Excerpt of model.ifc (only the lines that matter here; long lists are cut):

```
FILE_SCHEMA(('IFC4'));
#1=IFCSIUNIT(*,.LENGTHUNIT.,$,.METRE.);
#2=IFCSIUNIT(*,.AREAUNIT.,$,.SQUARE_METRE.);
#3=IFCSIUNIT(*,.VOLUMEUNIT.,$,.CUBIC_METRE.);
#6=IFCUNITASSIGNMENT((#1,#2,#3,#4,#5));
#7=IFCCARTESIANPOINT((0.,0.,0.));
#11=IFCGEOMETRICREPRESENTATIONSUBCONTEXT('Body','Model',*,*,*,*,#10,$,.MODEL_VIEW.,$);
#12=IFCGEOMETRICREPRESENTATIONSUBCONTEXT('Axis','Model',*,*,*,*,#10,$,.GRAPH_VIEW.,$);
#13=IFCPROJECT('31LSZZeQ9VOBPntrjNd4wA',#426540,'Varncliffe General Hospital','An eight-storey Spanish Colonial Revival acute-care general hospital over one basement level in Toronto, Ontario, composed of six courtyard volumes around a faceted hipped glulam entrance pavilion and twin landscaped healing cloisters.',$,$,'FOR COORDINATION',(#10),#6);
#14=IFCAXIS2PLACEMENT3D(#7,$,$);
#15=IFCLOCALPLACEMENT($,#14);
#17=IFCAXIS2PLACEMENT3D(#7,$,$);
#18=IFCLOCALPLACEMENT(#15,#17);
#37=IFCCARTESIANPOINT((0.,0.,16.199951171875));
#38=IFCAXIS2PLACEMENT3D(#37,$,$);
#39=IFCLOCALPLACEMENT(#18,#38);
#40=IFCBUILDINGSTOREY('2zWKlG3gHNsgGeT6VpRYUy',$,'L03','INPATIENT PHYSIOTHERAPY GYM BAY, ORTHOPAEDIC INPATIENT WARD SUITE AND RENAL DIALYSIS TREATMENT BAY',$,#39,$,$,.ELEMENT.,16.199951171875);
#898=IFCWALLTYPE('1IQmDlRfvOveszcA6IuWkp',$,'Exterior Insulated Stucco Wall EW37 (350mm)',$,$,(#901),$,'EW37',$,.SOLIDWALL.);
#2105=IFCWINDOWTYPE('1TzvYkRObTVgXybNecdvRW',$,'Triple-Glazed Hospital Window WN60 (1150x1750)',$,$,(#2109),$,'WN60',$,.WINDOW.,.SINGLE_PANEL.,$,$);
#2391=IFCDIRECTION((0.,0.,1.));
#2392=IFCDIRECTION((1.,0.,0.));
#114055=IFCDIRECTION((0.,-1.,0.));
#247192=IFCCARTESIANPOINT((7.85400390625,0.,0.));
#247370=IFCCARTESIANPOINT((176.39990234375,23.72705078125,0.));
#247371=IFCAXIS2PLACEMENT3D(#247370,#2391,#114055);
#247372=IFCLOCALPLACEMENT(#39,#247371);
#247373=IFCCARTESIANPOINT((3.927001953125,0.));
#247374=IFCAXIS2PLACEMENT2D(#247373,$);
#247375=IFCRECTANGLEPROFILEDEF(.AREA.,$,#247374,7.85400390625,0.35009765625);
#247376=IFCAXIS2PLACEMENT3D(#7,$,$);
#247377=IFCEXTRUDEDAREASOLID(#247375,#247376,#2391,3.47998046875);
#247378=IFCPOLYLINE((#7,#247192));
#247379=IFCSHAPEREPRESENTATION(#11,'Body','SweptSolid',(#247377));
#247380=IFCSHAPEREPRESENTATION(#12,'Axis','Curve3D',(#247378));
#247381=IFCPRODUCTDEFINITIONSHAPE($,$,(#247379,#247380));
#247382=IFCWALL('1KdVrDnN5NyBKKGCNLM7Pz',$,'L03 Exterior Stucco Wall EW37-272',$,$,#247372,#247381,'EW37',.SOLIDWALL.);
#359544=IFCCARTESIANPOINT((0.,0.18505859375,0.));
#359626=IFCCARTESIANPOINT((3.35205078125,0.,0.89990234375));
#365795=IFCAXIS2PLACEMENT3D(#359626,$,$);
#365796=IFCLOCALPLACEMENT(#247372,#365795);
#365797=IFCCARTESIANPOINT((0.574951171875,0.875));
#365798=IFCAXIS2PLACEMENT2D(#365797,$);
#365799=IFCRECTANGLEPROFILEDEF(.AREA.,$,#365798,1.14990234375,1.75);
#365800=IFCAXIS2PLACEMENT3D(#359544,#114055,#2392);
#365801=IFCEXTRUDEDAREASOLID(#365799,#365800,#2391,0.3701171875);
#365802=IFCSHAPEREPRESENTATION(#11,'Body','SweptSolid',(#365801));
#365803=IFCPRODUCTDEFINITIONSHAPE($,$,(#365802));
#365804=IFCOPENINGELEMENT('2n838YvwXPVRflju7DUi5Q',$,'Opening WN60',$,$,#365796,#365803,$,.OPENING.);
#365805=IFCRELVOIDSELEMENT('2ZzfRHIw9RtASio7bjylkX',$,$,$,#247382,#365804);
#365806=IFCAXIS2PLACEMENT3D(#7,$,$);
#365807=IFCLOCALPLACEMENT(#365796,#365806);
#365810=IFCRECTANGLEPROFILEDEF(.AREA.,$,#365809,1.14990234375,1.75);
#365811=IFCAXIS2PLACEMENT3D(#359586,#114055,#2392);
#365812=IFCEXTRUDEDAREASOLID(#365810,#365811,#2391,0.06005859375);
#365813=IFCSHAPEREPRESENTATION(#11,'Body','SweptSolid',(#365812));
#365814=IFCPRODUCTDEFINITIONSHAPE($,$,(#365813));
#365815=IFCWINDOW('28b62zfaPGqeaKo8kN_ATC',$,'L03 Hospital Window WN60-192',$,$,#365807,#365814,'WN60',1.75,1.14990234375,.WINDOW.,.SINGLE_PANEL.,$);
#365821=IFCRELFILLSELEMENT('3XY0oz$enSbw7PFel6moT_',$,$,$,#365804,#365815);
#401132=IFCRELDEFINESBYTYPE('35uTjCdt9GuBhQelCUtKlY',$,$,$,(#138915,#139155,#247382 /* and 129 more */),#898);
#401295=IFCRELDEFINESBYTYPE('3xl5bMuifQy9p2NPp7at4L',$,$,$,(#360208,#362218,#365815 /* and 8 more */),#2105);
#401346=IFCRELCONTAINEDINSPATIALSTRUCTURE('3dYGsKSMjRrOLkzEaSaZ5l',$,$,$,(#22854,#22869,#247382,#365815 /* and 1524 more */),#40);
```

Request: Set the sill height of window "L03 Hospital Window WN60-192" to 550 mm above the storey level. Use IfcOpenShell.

```python
import numpy as np
import ifcopenshell
import ifcopenshell.api.geometry
import ifcopenshell.geom
import ifcopenshell.util.element
import ifcopenshell.util.placement
import ifcopenshell.util.shape
import ifcopenshell.util.unit

model = ifcopenshell.open("model.ifc")
unit_scale = ifcopenshell.util.unit.calculate_unit_scale(model)

window = model.by_guid("28b62zfaPGqeaKo8kN_ATC")
opening = window.FillsVoids[0].RelatingOpeningElement
storey = ifcopenshell.util.element.get_container(window, ifc_class="IfcBuildingStorey")
level = ifcopenshell.util.placement.get_local_placement(storey.ObjectPlacement)[2, 3]

# The opening's origin need not be at the sill, so measure its lowest point.
shape = ifcopenshell.geom.create_shape(ifcopenshell.geom.settings(), opening)
bottom = ifcopenshell.util.shape.get_shape_bottom_elevation(shape, shape.geometry) / unit_scale
dz = level + 0.55 / unit_scale - bottom

shift = np.array([0.0, 0.0, dz])
# The window is placed relative to its opening, so it follows when the opening moves.
matrix = ifcopenshell.util.placement.get_local_placement(opening.ObjectPlacement)
matrix[:3, 3] += shift
ifcopenshell.api.geometry.edit_object_placement(
    model, product=opening, matrix=matrix, is_si=False, should_transform_children=True
)

print(f"moved by {dz * unit_scale:+.3f} m")

model.write("model_updated.ifc")
```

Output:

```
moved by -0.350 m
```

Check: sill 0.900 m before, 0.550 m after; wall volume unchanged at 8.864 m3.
